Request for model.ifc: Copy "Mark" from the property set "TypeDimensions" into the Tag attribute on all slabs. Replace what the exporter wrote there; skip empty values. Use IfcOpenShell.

First a look at what the model holds.

```python
import ifcopenshell
import ifcopenshell.util.element

model = ifcopenshell.open("model.ifc")
print(model.schema)
slabs = model.by_type("IfcSlab")
print(len(slabs), "slabs")
for e in slabs[:8]:
    source = ifcopenshell.util.element.get_pset(e, "TypeDimensions", "Mark")
    target = e.Tag
    print(e.id(), repr(source), repr(target), sep=" | ")
```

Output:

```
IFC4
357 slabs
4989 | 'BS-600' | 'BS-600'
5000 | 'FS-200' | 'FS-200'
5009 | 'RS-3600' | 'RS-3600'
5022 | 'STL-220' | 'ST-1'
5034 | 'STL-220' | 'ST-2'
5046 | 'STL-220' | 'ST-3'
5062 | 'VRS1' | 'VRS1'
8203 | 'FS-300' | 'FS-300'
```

```python
import ifcopenshell
import ifcopenshell.util.element

model = ifcopenshell.open("model.ifc")

count = 0
for e in model.by_type("IfcSlab"):
    value = ifcopenshell.util.element.get_pset(e, "TypeDimensions", "Mark")
    current = e.Tag
    if not value or not value.strip() or current == value:
        continue
    e.Tag = value
    count += 1

print(count, "slabs updated")

model.write("model-out.ifc")
```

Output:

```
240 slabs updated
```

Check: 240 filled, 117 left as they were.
